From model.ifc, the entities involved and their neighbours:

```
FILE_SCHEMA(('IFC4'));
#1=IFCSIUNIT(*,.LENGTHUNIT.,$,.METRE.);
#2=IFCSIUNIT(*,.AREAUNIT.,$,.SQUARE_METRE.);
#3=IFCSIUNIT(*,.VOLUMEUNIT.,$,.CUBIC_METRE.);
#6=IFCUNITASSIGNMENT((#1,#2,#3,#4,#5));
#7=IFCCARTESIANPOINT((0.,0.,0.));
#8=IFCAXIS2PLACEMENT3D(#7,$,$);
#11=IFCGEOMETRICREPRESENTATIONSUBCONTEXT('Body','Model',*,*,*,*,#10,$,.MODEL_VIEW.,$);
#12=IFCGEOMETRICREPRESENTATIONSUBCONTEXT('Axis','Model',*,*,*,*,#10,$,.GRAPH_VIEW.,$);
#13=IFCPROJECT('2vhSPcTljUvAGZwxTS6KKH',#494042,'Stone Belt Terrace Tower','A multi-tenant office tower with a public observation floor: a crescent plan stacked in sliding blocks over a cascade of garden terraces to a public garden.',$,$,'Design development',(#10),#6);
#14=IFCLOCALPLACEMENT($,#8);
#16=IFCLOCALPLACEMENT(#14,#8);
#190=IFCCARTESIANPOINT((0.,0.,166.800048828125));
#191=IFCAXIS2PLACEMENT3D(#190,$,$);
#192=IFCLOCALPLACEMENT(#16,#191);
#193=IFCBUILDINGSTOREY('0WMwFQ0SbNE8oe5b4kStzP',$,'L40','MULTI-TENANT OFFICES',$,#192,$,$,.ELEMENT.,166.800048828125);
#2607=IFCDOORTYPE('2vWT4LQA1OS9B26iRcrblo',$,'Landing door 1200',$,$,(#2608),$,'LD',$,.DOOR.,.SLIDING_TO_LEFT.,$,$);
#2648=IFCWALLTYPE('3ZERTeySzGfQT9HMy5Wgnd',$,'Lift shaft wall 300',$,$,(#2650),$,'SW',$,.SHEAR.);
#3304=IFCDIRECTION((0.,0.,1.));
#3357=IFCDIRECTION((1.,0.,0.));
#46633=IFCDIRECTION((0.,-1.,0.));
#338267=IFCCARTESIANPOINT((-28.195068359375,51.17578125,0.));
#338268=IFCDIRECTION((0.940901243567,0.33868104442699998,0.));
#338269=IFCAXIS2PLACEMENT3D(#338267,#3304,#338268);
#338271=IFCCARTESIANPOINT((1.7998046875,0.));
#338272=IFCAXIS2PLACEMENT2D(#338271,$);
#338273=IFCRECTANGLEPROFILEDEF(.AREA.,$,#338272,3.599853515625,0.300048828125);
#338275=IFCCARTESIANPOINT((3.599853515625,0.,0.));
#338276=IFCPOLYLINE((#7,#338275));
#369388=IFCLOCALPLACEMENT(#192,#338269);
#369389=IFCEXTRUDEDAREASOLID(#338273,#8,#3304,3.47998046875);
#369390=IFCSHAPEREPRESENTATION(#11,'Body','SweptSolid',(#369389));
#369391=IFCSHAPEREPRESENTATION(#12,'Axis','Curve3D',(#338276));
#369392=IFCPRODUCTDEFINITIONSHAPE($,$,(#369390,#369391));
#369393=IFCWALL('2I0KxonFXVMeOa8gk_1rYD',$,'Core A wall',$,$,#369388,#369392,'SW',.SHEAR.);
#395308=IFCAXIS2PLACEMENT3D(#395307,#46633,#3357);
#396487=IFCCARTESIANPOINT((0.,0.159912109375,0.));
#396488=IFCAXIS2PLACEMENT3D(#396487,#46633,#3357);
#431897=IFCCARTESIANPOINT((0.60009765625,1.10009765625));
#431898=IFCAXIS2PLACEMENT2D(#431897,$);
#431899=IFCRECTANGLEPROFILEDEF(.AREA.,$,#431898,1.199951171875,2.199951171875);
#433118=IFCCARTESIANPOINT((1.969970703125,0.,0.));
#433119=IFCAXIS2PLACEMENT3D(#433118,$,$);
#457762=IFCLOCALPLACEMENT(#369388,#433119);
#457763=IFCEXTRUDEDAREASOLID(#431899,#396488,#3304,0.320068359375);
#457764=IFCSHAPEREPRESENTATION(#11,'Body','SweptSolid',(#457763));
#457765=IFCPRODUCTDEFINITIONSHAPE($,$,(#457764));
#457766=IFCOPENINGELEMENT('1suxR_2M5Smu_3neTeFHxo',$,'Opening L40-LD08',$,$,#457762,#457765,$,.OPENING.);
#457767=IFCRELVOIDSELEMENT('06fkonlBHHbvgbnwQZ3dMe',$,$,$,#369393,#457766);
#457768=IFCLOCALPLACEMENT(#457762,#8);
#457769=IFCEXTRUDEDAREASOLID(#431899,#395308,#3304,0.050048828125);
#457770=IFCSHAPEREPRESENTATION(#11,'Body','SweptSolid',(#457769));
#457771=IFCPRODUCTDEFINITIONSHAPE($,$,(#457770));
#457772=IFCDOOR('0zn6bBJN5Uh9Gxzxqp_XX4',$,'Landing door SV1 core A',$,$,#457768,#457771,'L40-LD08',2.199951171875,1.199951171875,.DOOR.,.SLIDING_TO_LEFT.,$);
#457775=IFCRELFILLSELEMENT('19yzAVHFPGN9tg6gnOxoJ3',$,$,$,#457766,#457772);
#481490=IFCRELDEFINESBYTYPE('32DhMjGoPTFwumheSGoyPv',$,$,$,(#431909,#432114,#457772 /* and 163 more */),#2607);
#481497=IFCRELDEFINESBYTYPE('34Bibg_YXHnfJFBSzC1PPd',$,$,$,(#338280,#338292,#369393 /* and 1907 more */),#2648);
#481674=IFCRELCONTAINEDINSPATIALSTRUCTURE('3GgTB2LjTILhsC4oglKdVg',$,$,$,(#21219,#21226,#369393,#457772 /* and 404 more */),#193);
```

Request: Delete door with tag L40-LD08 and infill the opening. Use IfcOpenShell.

```python
import ifcopenshell
import ifcopenshell.api.feature
import ifcopenshell.api.root
import ifcopenshell.geom
import ifcopenshell.util.shape

model = ifcopenshell.open("model.ifc")
settings = ifcopenshell.geom.settings()


def volume(element):
    """Net volume in cubic metres, openings subtracted."""
    shape = ifcopenshell.geom.create_shape(settings, element)
    return ifcopenshell.util.shape.get_volume(shape.geometry)


door = model.by_id(457772)
opening = door.FillsVoids[0].RelatingOpeningElement
wall = opening.VoidsElements[0].RelatingBuildingElement
before = volume(wall)

ifcopenshell.api.root.remove_product(model, product=door)
ifcopenshell.api.feature.remove_feature(model, feature=opening)

after = volume(wall)

print(f"wall volume {before:.3f} -> {after:.3f} m3")

model.write("model_updated.ifc")
```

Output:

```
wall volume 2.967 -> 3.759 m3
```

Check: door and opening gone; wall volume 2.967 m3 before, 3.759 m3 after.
